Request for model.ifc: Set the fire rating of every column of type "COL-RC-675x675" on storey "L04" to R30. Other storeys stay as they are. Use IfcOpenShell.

First a look at what the model holds.

```python
import ifcopenshell
import ifcopenshell.util.element

model = ifcopenshell.open("model.ifc")
print(model.schema)
storey = next(s for s in model.by_type("IfcBuildingStorey") if s.Name == "L04")
columns = [e for e in ifcopenshell.util.element.get_decomposition(storey) if e.is_a("IfcColumn")]
seen = {}
for e in columns:
    element_type = ifcopenshell.util.element.get_type(e)
    key = (element_type.Name if element_type != e and element_type else None, ifcopenshell.util.element.get_pset(e, "Pset_ColumnCommon", "FireRating"))
    seen[key] = seen.get(key, 0) + 1
for (name, value), count in sorted(seen.items(), key=str):
    print(count, "x", name, "|", value)
```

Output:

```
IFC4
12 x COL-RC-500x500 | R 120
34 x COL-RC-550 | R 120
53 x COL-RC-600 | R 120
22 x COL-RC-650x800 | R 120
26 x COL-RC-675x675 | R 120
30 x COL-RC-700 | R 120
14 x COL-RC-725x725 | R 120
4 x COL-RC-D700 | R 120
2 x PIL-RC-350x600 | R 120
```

```python
import ifcopenshell
import ifcopenshell.api.pset
import ifcopenshell.util.element

model = ifcopenshell.open("model.ifc")

storey = next(s for s in model.by_type("IfcBuildingStorey") if s.Name == "L04")
columns = [e for e in ifcopenshell.util.element.get_decomposition(storey) if e.is_a("IfcColumn")]

count = 0
for e in columns:
    element_type = ifcopenshell.util.element.get_type(e)
    if element_type in (None, e) or element_type.Name != "COL-RC-675x675":
        continue
    # add_pset returns the element's existing set when there is one.
    pset = ifcopenshell.api.pset.add_pset(model, product=e, name="Pset_ColumnCommon")
    ifcopenshell.api.pset.edit_pset(model, pset=pset, properties={"FireRating": "R30"})
    count += 1

print(count, "columns updated")

model.write("model_edited.ifc")
```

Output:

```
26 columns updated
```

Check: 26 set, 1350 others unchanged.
